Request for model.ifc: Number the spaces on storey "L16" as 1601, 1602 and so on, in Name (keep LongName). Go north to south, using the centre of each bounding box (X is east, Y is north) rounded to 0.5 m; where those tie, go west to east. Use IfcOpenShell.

First a look at what the model holds.

```python
import ifcopenshell
import ifcopenshell.util.element
import ifcopenshell.util.placement

model = ifcopenshell.open("model.ifc")
print(model.schema)
storey = next(s for s in model.by_type("IfcBuildingStorey") if s.Name == "L16")
spaces = [e for e in ifcopenshell.util.element.get_decomposition(storey) if e.is_a("IfcSpace")]
for e in sorted(spaces, key=lambda e: e.id()):
    origin = ifcopenshell.util.placement.get_local_placement(e.ObjectPlacement)[:3, 3]
    print(e.id(), e.Name, e.LongName, origin.round(2) + 0.0, sep=" | ")
```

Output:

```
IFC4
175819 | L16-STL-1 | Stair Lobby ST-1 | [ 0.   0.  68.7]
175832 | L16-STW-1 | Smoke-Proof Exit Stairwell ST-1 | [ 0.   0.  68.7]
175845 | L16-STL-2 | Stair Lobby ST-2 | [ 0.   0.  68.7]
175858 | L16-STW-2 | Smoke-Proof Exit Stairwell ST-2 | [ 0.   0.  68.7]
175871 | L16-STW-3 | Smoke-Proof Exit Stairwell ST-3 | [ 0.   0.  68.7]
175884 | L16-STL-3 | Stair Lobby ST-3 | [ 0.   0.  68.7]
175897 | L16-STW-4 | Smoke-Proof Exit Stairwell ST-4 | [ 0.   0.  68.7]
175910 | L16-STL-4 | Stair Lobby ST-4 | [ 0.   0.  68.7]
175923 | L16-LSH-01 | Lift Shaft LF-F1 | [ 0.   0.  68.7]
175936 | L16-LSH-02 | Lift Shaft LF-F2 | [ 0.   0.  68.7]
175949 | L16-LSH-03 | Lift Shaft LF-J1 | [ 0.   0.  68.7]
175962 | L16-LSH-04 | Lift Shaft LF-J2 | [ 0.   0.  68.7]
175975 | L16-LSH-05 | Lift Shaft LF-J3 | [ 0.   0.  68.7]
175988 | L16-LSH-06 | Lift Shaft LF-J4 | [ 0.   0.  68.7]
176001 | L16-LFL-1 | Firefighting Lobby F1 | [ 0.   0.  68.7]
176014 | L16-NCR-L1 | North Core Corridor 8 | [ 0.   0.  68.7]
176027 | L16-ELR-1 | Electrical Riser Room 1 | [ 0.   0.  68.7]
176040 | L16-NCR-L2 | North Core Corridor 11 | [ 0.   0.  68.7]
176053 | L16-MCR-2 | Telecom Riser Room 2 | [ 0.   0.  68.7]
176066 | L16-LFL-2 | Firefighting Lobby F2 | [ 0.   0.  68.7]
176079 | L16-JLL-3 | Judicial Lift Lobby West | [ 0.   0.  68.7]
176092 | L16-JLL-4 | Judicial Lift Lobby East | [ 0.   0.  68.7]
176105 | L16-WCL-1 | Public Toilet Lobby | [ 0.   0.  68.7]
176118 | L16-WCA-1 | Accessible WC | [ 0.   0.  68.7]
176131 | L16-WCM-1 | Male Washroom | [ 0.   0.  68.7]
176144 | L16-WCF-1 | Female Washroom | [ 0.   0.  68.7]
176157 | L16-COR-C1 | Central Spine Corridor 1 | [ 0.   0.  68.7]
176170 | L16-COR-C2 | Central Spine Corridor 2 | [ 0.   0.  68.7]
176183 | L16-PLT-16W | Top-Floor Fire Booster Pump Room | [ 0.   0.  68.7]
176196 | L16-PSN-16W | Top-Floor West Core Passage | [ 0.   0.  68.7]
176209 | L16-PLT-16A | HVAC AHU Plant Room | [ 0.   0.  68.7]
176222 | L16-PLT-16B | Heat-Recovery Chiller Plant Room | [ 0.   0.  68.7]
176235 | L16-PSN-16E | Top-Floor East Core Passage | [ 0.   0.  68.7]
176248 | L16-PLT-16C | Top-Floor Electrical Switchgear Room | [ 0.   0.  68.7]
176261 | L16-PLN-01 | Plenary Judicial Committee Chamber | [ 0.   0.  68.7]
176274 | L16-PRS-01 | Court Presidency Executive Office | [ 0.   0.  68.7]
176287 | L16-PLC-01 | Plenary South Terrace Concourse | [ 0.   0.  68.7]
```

```python
import ifcopenshell
import ifcopenshell.geom
import ifcopenshell.util.element
import ifcopenshell.util.shape

model = ifcopenshell.open("model.ifc")
settings = ifcopenshell.geom.settings()
settings.set("use-world-coords", True)


def centre(element):
    shape = ifcopenshell.geom.create_shape(settings, element)
    return ifcopenshell.util.shape.get_bbox_centroid(shape.geometry)


storey = next(s for s in model.by_type("IfcBuildingStorey") if s.Name == "L16")
spaces = [e for e in ifcopenshell.util.element.get_decomposition(storey) if e.is_a("IfcSpace")]

# Insertion points can sit at a corner or the storey origin, so sort by the geometry (in metres).
centres = {e: centre(e) for e in spaces}
spaces.sort(key=lambda e: (-round(centres[e][1] / 0.5), centres[e][0]))

for i, e in enumerate(spaces, start=1):
    number = f"16{i:02d}"
    e.Name = number
    print(e.id(), number)

model.write("model_edited.ifc")
```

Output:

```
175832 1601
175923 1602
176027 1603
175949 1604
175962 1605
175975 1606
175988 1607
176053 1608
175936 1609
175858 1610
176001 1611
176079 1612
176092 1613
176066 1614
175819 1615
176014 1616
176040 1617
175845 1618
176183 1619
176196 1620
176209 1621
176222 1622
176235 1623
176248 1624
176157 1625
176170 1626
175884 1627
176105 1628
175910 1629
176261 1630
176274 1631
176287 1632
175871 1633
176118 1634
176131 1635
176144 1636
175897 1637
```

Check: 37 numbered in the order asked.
